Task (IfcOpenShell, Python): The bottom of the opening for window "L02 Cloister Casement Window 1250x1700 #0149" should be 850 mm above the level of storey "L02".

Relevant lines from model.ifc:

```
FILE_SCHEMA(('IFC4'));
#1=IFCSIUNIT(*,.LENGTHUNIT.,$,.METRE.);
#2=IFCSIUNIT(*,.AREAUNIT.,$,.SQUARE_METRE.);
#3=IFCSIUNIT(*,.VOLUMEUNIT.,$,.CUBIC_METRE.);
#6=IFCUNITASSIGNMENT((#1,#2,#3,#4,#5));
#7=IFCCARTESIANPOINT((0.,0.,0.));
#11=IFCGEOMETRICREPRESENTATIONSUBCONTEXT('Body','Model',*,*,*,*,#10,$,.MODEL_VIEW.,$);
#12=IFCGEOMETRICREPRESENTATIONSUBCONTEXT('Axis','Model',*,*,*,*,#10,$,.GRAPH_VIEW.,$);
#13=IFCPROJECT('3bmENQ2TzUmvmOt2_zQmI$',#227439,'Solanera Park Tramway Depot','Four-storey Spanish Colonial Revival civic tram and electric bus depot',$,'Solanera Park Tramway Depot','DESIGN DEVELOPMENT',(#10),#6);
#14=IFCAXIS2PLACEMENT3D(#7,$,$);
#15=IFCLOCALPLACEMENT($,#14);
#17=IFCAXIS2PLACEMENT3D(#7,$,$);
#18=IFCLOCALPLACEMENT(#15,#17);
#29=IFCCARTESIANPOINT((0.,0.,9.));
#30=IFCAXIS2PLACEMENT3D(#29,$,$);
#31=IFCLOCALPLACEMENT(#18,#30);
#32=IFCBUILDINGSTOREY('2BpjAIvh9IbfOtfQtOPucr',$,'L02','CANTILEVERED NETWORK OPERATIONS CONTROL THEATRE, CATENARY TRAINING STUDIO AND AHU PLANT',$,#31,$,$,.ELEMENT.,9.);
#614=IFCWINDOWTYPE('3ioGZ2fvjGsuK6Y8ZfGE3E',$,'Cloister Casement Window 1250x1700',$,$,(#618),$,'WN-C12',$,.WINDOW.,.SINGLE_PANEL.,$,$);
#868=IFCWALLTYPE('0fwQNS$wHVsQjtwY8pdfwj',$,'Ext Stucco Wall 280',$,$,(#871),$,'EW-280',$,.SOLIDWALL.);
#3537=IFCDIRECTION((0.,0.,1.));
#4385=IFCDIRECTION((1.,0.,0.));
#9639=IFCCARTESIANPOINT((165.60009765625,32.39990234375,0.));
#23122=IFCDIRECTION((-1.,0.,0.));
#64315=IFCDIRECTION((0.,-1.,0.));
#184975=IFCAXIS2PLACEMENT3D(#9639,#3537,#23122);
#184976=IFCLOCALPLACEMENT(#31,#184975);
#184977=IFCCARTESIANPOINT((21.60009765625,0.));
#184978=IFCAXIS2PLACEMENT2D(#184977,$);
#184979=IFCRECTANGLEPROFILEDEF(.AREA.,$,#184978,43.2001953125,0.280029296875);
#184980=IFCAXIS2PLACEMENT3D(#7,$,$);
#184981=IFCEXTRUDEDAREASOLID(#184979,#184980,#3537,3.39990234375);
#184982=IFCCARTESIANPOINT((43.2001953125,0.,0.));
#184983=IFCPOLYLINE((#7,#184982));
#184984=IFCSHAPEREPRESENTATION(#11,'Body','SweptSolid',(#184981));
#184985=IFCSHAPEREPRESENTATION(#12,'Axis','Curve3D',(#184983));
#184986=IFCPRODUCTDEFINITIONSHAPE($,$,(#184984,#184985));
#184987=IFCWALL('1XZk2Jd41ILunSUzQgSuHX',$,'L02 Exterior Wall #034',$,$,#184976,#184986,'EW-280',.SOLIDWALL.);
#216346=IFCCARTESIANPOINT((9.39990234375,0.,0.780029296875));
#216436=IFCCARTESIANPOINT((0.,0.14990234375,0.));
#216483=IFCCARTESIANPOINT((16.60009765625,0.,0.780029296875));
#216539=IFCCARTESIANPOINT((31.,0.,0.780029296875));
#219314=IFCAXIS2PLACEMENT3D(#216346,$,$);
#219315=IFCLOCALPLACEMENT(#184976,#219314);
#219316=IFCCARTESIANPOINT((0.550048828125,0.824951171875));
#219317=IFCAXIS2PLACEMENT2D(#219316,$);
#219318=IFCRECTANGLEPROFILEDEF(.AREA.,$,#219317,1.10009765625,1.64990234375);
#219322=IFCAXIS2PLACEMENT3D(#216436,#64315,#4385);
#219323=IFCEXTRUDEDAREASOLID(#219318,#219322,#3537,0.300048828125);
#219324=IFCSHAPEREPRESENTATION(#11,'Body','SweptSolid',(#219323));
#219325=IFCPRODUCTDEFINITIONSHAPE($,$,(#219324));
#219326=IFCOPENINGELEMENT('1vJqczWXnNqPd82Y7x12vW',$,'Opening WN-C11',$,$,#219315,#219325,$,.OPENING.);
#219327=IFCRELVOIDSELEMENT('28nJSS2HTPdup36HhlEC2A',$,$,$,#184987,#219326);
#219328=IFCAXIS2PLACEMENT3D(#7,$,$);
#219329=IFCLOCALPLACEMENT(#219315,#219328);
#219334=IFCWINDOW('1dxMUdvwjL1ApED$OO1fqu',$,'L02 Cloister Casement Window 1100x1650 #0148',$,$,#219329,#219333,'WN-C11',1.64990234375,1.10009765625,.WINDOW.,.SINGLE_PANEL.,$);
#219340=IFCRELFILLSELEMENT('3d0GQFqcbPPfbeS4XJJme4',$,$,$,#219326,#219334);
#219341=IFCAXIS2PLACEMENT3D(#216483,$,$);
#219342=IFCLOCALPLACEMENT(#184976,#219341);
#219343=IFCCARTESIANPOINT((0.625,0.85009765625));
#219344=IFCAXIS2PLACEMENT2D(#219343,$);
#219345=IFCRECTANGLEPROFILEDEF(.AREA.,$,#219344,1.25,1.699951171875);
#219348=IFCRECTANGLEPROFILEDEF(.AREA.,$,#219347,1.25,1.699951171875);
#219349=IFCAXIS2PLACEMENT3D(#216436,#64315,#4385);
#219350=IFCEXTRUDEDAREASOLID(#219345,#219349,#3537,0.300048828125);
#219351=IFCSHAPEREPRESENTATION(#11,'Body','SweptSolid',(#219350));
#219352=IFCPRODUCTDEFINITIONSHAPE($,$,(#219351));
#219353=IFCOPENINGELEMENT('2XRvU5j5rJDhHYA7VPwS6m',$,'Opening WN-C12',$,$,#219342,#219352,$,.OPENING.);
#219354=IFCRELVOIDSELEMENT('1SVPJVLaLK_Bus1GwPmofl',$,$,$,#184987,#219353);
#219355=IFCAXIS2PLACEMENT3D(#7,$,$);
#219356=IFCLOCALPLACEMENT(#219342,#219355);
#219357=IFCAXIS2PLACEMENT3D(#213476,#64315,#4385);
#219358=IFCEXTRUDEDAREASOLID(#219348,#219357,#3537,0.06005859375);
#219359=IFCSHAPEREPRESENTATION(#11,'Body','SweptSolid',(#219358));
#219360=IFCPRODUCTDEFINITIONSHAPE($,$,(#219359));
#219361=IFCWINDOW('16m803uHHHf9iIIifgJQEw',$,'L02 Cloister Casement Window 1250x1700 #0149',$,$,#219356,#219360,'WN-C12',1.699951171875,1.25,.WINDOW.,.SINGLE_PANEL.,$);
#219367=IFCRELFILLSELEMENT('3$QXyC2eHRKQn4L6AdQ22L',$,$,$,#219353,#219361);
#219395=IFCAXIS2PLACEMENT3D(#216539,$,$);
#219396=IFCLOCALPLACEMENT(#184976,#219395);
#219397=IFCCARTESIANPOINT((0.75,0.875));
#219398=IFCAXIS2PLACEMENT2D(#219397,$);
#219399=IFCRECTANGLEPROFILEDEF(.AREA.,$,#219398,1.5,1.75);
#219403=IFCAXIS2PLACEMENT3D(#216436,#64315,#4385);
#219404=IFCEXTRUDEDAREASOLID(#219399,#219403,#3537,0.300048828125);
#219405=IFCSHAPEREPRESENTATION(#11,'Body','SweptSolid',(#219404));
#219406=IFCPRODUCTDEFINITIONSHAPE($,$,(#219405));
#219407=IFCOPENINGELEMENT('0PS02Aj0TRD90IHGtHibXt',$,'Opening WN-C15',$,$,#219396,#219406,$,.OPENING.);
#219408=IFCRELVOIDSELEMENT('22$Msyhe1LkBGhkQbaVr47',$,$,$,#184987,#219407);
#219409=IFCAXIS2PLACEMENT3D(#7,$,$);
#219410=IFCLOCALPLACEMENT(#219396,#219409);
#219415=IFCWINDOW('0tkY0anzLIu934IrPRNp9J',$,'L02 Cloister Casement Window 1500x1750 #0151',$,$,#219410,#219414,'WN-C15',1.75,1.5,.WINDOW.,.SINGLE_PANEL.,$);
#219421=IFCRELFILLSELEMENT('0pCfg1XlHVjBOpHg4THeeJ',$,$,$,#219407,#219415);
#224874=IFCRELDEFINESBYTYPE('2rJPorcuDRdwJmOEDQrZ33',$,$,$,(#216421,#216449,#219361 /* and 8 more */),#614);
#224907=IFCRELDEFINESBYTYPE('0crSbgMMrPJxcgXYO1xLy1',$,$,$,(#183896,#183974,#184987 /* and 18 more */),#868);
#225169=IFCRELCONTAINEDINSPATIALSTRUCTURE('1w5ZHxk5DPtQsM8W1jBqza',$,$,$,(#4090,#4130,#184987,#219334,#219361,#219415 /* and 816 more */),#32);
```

```python
import numpy as np
import ifcopenshell
import ifcopenshell.api.geometry
import ifcopenshell.geom
import ifcopenshell.util.element
import ifcopenshell.util.placement
import ifcopenshell.util.shape
import ifcopenshell.util.unit

model = ifcopenshell.open("model.ifc")
unit_scale = ifcopenshell.util.unit.calculate_unit_scale(model)

window = model.by_guid("16m803uHHHf9iIIifgJQEw")
opening = window.FillsVoids[0].RelatingOpeningElement
storey = ifcopenshell.util.element.get_container(window, ifc_class="IfcBuildingStorey")
level = ifcopenshell.util.placement.get_local_placement(storey.ObjectPlacement)[2, 3]

# The opening's origin need not be at the sill, so measure its lowest point.
shape = ifcopenshell.geom.create_shape(ifcopenshell.geom.settings(), opening)
bottom = ifcopenshell.util.shape.get_shape_bottom_elevation(shape, shape.geometry) / unit_scale
dz = level + 0.85 / unit_scale - bottom

shift = np.array([0.0, 0.0, dz])
# The window is placed relative to its opening, so it follows when the opening moves.
matrix = ifcopenshell.util.placement.get_local_placement(opening.ObjectPlacement)
matrix[:3, 3] += shift
ifcopenshell.api.geometry.edit_object_placement(
    model, product=opening, matrix=matrix, is_si=False, should_transform_children=True
)

print(f"moved by {dz * unit_scale:+.3f} m")

model.write("model_edited.ifc")
```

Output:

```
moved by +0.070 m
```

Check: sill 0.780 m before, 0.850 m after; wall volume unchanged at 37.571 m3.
